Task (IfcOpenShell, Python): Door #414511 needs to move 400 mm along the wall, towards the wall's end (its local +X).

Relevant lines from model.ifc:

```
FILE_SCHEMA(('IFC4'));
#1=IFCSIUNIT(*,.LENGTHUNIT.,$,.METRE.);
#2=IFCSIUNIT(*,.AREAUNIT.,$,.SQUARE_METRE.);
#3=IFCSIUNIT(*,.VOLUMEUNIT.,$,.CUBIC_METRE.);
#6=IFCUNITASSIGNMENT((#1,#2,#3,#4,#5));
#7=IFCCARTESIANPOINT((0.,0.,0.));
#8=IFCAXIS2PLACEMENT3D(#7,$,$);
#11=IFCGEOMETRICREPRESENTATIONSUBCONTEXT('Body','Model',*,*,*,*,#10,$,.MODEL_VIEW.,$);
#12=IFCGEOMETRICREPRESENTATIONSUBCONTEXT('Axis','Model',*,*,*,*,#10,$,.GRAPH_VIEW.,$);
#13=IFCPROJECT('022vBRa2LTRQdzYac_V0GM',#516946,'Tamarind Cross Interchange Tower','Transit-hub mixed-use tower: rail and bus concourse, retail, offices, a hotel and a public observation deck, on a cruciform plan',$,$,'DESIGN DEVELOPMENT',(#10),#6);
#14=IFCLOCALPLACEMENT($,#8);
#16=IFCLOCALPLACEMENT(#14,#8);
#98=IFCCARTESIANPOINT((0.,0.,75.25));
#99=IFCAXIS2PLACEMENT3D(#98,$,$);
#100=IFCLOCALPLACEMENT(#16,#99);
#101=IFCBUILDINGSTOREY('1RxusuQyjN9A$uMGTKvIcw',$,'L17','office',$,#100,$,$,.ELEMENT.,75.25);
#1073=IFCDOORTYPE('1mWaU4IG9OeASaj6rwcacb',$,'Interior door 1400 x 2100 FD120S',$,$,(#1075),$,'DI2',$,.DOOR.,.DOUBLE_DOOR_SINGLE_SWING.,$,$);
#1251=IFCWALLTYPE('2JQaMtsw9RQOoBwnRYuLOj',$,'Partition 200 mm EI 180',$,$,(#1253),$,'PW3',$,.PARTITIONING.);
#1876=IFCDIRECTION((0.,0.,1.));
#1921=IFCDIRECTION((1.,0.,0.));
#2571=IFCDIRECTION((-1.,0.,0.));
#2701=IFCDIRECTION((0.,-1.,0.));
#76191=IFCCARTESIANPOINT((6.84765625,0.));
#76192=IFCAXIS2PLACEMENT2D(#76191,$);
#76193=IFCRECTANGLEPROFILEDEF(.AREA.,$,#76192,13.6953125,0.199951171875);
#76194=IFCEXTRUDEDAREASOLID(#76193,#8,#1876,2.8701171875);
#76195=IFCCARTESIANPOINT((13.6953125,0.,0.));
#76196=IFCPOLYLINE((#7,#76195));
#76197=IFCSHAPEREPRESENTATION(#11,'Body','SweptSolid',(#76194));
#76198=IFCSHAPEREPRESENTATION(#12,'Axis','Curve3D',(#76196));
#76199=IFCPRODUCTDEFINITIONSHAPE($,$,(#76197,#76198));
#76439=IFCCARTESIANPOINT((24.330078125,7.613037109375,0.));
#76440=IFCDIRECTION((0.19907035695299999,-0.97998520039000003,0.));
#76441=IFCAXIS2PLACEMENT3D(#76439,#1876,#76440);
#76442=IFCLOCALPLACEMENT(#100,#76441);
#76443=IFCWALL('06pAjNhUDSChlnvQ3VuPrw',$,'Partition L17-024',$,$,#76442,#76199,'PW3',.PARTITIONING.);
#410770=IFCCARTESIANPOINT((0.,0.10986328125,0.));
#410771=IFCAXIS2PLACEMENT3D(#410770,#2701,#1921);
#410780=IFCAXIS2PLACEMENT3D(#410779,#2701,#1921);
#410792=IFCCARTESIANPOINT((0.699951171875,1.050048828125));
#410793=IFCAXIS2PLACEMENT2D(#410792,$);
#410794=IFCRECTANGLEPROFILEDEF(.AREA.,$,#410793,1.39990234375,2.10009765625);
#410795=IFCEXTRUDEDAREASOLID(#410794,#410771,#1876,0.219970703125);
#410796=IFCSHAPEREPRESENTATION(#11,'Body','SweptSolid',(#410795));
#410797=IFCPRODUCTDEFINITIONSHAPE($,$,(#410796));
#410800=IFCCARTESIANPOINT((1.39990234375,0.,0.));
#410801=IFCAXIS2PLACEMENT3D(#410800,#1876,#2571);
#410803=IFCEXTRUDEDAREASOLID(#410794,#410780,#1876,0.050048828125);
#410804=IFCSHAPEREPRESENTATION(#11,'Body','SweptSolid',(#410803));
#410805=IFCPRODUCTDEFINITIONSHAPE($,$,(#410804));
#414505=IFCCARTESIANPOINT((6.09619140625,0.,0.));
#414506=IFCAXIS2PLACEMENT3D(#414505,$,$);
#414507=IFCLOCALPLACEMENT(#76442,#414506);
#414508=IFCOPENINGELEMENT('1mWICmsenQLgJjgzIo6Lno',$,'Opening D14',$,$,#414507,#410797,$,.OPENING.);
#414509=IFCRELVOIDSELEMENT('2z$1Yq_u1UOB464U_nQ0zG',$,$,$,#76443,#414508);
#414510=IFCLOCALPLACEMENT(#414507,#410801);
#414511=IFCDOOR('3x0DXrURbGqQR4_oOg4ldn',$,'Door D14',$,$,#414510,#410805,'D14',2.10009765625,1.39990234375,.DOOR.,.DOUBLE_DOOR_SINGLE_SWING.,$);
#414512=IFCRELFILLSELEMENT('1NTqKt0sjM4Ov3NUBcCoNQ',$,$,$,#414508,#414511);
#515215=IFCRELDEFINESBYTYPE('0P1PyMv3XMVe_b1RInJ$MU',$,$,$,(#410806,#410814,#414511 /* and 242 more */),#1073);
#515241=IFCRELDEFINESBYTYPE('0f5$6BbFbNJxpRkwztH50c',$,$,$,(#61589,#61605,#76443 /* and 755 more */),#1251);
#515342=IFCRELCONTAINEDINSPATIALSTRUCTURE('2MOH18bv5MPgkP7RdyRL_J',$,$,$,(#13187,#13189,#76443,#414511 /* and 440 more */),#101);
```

```python
import ifcopenshell
import ifcopenshell.api.geometry
import ifcopenshell.util.placement
import ifcopenshell.util.unit

model = ifcopenshell.open("model.ifc")
unit_scale = ifcopenshell.util.unit.calculate_unit_scale(model)

door = model.by_guid("3x0DXrURbGqQR4_oOg4ldn")
opening = door.FillsVoids[0].RelatingOpeningElement
wall = opening.VoidsElements[0].RelatingBuildingElement

wall_matrix = ifcopenshell.util.placement.get_local_placement(wall.ObjectPlacement)
shift = wall_matrix[:3, 0] * 0.4 / unit_scale
before = ifcopenshell.util.placement.get_local_placement(door.ObjectPlacement)[:3, 3].copy()

# The door is placed relative to its opening, so it follows when the opening moves.
matrix = ifcopenshell.util.placement.get_local_placement(opening.ObjectPlacement)
matrix[:3, 3] += shift
ifcopenshell.api.geometry.edit_object_placement(
    model, product=opening, matrix=matrix, is_si=False, should_transform_children=True
)

after = ifcopenshell.util.placement.get_local_placement(door.ObjectPlacement)[:3, 3]
print("door moved by", (after - before).round(3) + 0.0)

model.write("model_v2.ifc")
```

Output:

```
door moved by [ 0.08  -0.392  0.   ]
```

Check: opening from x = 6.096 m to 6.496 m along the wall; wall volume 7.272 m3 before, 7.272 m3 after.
